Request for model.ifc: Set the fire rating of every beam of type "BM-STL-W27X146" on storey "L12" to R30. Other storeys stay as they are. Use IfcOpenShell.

First a look at what the model holds.

```python
import ifcopenshell
import ifcopenshell.util.element

model = ifcopenshell.open("model.ifc")
print(model.schema)
storey = next(s for s in model.by_type("IfcBuildingStorey") if s.Name == "L12")
beams = [e for e in ifcopenshell.util.element.get_decomposition(storey) if e.is_a("IfcBeam")]
seen = {}
for e in beams:
    element_type = ifcopenshell.util.element.get_type(e)
    key = (element_type.Name if element_type != e and element_type else None, ifcopenshell.util.element.get_pset(e, "Pset_BeamCommon", "FireRating"))
    seen[key] = seen.get(key, 0) + 1
for (name, value), count in sorted(seen.items(), key=str):
    print(count, "x", name, "|", value)
```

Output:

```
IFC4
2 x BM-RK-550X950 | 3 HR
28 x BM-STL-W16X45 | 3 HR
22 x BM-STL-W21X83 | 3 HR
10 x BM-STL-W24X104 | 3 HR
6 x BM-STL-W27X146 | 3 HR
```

```python
import ifcopenshell
import ifcopenshell.api.pset
import ifcopenshell.util.element

model = ifcopenshell.open("model.ifc")

storey = next(s for s in model.by_type("IfcBuildingStorey") if s.Name == "L12")
beams = [e for e in ifcopenshell.util.element.get_decomposition(storey) if e.is_a("IfcBeam")]

count = 0
for e in beams:
    element_type = ifcopenshell.util.element.get_type(e)
    if element_type in (None, e) or element_type.Name != "BM-STL-W27X146":
        continue
    # add_pset returns the element's existing set when there is one.
    pset = ifcopenshell.api.pset.add_pset(model, product=e, name="Pset_BeamCommon")
    ifcopenshell.api.pset.edit_pset(model, pset=pset, properties={"FireRating": "R30"})
    count += 1

print(count, "beams updated")

model.write("model_rev.ifc")
```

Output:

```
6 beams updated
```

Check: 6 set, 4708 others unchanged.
